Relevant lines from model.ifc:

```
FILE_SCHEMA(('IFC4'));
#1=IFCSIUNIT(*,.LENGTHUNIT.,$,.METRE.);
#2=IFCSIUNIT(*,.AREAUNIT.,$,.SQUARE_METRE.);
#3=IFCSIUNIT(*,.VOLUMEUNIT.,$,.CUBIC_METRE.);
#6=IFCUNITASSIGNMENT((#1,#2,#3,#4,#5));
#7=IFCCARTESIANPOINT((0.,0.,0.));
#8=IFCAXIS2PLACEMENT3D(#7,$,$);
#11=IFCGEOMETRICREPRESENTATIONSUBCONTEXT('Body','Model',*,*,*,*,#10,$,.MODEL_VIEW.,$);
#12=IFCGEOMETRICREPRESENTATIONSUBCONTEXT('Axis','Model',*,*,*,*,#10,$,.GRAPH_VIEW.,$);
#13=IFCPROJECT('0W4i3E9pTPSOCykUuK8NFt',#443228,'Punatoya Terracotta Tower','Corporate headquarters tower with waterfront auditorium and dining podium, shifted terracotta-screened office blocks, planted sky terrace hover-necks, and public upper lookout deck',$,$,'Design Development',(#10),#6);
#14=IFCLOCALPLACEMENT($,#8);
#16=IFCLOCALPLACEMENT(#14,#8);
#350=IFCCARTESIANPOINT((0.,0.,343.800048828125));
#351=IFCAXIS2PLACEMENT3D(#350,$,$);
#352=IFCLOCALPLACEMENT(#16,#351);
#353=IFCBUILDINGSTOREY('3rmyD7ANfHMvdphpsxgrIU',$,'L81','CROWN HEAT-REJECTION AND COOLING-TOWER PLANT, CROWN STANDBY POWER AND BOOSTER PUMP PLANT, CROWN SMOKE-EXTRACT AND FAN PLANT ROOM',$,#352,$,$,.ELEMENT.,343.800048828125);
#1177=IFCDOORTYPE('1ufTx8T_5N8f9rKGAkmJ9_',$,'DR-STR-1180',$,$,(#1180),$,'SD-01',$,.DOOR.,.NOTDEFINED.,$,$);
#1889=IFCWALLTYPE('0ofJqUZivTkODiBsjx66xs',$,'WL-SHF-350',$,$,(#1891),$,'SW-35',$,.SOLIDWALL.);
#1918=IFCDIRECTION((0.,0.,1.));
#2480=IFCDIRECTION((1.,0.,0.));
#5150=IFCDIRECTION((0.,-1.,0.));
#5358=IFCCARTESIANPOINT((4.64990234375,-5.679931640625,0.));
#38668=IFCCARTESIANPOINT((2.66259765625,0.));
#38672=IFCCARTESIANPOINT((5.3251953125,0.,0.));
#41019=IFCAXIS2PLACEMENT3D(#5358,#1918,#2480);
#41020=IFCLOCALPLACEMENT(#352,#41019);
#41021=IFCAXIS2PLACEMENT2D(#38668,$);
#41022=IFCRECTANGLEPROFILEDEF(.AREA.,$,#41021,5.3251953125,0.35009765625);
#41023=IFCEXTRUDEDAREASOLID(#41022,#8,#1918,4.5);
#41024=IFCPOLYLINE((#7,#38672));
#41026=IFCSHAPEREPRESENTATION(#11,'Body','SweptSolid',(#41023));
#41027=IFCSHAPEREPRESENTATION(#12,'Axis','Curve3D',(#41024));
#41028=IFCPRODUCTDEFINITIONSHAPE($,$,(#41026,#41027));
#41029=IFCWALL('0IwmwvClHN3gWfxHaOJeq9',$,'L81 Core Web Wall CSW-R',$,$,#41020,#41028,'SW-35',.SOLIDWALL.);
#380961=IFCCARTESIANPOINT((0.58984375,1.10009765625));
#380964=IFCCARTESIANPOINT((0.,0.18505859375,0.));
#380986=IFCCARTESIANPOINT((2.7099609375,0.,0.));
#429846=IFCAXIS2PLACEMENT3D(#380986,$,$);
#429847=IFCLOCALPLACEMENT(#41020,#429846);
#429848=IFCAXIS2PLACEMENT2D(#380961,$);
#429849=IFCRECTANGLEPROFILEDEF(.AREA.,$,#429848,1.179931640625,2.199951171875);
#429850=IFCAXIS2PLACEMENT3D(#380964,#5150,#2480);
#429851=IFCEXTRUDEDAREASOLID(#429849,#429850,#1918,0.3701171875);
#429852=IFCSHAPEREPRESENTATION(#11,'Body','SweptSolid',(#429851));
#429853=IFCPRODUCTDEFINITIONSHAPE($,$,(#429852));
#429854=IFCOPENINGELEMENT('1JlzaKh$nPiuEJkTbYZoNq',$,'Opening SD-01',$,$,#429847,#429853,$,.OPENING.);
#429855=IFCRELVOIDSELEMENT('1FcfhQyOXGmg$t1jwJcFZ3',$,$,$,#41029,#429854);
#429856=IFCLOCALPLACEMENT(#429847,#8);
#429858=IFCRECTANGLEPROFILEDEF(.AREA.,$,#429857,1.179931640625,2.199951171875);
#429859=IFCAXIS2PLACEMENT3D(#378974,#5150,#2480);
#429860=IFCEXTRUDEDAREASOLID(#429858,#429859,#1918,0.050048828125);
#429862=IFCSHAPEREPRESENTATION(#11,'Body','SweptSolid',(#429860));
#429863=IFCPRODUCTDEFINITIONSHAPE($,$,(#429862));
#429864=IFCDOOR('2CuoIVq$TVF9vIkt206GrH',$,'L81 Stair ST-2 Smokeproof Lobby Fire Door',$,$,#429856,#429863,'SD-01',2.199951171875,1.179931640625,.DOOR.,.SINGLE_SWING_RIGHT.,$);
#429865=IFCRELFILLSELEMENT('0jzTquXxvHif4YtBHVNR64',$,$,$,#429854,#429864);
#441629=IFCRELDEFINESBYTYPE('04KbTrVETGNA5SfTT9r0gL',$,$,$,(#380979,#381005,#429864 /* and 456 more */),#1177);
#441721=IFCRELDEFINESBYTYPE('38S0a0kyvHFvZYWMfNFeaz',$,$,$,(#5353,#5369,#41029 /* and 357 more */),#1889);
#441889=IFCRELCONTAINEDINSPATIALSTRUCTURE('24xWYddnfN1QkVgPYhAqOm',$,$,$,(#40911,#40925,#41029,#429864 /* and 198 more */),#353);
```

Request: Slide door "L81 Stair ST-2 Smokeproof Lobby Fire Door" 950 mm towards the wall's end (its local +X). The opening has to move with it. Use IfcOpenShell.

```python
import ifcopenshell
import ifcopenshell.api.geometry
import ifcopenshell.util.placement
import ifcopenshell.util.unit

model = ifcopenshell.open("model.ifc")
unit_scale = ifcopenshell.util.unit.calculate_unit_scale(model)

door = model.by_guid("2CuoIVq$TVF9vIkt206GrH")
opening = door.FillsVoids[0].RelatingOpeningElement
wall = opening.VoidsElements[0].RelatingBuildingElement

wall_matrix = ifcopenshell.util.placement.get_local_placement(wall.ObjectPlacement)
shift = wall_matrix[:3, 0] * 0.95 / unit_scale
before = ifcopenshell.util.placement.get_local_placement(door.ObjectPlacement)[:3, 3].copy()

# The door is placed relative to its opening, so it follows when the opening moves.
matrix = ifcopenshell.util.placement.get_local_placement(opening.ObjectPlacement)
matrix[:3, 3] += shift
ifcopenshell.api.geometry.edit_object_placement(
    model, product=opening, matrix=matrix, is_si=False, should_transform_children=True
)

after = ifcopenshell.util.placement.get_local_placement(door.ObjectPlacement)[:3, 3]
print("door moved by", (after - before).round(3) + 0.0)

model.write("model_updated.ifc")
```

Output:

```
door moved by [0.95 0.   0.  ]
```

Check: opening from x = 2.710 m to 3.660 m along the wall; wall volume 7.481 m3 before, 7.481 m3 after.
